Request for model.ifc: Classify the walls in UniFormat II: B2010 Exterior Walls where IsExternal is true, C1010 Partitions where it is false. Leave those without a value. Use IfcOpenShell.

First a look at what the model holds.

```python
import ifcopenshell
import ifcopenshell.util.element

model = ifcopenshell.open("model.ifc")
print(model.schema)
print("classifications:", [c.Name for c in model.by_type("IfcClassification")])
values = [ifcopenshell.util.element.get_pset(e, "Pset_WallCommon", "IsExternal") for e in model.by_type("IfcWall")]
for value in (True, False, None):
    print("IsExternal", value, values.count(value))
```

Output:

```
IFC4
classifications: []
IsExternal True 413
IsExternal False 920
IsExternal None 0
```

```python
import ifcopenshell
import ifcopenshell.api.classification
import ifcopenshell.util.element

model = ifcopenshell.open("model.ifc")

system = ifcopenshell.api.classification.add_classification(model, classification="UniFormat II")

walls = model.by_type("IfcWall")
external = {e: ifcopenshell.util.element.get_pset(e, "Pset_WallCommon", "IsExternal") for e in walls}
for flag, code, name in ((True, "B2010", "Exterior Walls"), (False, "C1010", "Partitions")):
    products = [e for e in walls if external[e] is flag]
    ifcopenshell.api.classification.add_reference(
        model, products=products, classification=system, identification=code, name=name
    )
    print(code, len(products))

model.write("model_edited.ifc")
```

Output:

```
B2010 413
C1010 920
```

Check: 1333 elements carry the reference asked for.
